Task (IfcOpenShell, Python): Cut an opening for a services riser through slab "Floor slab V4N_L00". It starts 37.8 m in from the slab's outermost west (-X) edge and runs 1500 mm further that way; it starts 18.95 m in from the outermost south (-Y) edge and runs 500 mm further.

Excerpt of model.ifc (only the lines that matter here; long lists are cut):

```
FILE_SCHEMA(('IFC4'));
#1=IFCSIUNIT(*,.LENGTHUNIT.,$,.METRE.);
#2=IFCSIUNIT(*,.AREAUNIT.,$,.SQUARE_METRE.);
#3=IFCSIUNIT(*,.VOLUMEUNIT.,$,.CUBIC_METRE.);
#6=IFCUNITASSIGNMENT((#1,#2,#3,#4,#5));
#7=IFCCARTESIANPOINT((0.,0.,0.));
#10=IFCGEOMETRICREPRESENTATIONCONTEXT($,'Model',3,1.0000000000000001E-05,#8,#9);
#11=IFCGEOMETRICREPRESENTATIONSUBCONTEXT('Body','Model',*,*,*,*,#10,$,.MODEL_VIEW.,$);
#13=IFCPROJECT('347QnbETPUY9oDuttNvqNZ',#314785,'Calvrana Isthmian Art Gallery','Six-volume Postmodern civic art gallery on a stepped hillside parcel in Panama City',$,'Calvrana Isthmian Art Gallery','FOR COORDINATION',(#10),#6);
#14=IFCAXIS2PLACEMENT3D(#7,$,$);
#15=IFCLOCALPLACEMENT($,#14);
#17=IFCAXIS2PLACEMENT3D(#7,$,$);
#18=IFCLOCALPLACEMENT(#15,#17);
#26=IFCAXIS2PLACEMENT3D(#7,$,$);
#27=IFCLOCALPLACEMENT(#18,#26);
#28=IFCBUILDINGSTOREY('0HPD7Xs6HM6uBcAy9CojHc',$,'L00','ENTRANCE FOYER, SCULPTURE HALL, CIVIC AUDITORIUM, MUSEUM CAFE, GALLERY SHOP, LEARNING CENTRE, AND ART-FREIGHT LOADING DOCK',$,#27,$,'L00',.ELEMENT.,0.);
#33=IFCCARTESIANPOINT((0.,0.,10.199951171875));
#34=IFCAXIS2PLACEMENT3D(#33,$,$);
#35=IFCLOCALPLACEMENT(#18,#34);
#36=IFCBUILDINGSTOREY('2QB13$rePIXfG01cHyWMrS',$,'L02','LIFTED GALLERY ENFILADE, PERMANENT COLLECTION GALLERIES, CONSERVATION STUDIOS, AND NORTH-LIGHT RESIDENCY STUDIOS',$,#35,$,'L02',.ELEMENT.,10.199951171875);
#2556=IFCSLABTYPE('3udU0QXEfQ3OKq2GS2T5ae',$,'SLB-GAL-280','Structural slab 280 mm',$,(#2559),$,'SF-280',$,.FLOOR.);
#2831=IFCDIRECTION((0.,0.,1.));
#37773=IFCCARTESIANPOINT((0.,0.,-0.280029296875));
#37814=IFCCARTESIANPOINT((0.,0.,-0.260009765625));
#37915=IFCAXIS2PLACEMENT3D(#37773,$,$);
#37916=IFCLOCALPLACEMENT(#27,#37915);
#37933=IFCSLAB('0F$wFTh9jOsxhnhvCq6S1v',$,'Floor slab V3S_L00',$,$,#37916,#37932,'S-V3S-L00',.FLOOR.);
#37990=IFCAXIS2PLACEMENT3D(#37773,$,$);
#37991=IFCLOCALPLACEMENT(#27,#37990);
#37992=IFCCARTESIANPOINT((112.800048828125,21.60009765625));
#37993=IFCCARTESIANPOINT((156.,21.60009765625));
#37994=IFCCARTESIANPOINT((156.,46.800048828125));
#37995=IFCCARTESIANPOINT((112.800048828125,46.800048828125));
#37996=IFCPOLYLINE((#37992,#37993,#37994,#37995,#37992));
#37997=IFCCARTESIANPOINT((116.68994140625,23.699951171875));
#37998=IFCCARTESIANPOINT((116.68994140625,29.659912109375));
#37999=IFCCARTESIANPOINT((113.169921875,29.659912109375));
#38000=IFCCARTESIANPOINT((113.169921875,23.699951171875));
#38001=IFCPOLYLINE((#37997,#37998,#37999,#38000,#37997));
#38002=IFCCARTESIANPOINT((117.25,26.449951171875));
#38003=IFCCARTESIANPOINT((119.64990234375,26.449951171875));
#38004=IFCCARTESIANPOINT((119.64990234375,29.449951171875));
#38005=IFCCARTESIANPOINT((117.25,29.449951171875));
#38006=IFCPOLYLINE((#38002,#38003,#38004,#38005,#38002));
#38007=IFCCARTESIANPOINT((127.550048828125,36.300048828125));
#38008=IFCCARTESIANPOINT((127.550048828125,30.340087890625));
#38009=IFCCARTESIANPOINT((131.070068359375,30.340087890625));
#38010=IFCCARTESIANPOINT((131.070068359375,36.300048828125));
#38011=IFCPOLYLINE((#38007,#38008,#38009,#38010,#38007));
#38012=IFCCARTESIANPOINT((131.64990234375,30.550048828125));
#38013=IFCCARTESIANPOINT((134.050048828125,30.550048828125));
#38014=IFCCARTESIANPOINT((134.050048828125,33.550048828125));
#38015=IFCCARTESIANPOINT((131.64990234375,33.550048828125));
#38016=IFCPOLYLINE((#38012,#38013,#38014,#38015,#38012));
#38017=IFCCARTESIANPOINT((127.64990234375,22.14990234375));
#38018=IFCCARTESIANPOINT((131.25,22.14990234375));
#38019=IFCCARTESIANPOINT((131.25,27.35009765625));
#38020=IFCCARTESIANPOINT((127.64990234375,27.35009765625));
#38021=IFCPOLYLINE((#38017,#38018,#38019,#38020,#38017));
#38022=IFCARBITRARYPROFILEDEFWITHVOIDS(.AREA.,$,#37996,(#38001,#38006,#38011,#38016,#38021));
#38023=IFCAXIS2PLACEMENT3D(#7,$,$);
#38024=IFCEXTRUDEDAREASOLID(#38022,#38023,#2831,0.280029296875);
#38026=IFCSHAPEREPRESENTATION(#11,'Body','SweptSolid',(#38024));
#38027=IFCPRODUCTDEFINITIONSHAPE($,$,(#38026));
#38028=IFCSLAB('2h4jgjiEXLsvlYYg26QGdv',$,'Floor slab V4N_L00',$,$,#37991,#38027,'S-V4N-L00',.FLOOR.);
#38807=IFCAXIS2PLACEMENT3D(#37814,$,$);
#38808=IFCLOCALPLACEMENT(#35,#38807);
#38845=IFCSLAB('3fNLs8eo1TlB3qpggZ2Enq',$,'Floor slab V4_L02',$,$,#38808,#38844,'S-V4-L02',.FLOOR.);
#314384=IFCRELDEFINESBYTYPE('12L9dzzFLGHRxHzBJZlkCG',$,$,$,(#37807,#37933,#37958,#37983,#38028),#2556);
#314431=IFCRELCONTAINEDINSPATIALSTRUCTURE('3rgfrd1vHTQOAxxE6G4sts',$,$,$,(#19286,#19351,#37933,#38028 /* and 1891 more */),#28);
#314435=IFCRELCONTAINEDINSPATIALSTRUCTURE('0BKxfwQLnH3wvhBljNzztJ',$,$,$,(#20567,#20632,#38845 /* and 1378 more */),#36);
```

```python
import numpy as np
import ifcopenshell
import ifcopenshell.api.feature
import ifcopenshell.api.geometry
import ifcopenshell.api.root
import ifcopenshell.geom
import ifcopenshell.util.placement
import ifcopenshell.util.representation
import ifcopenshell.util.shape
import ifcopenshell.util.unit

model = ifcopenshell.open("model.ifc")
unit_scale = ifcopenshell.util.unit.calculate_unit_scale(model)
settings = ifcopenshell.geom.settings()


def volume(element):
    """Net volume in cubic metres, openings subtracted."""
    shape = ifcopenshell.geom.create_shape(settings, element)
    return ifcopenshell.util.shape.get_volume(shape.geometry)


slab = model.by_id(38028)
before = volume(slab)

# Extent in the slab's own axes, in metres. The edges named are its -X and -Y sides.
slab_shape = ifcopenshell.geom.create_shape(settings, slab)
vertices = ifcopenshell.util.shape.get_vertices(slab_shape.geometry)
x_min, y_min, bottom = vertices.min(axis=0)
top = vertices[:, 2].max()

opening = ifcopenshell.api.root.create_entity(model, ifc_class="IfcOpeningElement", name="Services riser opening", predefined_type="OPENING")
context = ifcopenshell.util.representation.get_context(model, "Model", "Body", "MODEL_VIEW")
width, depth = 1.5, 0.5
outline = [(0.0, 0.0), (width, 0.0), (width, depth), (0.0, depth), (0.0, 0.0)]
# Overshoot both faces by 50 mm so the cut is clean.
shape = ifcopenshell.api.geometry.add_slab_representation(
    model, context=context, depth=top - bottom + 0.1, polyline=outline
)
ifcopenshell.api.geometry.assign_representation(model, product=opening, representation=shape)

matrix = ifcopenshell.util.placement.get_local_placement(slab.ObjectPlacement)
matrix[:, 3] = matrix @ np.append(np.array([x_min + 37.8, y_min + 18.95, bottom - 0.05]) / unit_scale, 1.0)
ifcopenshell.api.geometry.edit_object_placement(model, product=opening, matrix=matrix, is_si=False)
ifcopenshell.api.feature.add_feature(model, feature=opening, element=slab)

after = volume(slab)

print(f"slab volume {before:.3f} -> {after:.3f} m3")

model.write("model_updated.ifc")
```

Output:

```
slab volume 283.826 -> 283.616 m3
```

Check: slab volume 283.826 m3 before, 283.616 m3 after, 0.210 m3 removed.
